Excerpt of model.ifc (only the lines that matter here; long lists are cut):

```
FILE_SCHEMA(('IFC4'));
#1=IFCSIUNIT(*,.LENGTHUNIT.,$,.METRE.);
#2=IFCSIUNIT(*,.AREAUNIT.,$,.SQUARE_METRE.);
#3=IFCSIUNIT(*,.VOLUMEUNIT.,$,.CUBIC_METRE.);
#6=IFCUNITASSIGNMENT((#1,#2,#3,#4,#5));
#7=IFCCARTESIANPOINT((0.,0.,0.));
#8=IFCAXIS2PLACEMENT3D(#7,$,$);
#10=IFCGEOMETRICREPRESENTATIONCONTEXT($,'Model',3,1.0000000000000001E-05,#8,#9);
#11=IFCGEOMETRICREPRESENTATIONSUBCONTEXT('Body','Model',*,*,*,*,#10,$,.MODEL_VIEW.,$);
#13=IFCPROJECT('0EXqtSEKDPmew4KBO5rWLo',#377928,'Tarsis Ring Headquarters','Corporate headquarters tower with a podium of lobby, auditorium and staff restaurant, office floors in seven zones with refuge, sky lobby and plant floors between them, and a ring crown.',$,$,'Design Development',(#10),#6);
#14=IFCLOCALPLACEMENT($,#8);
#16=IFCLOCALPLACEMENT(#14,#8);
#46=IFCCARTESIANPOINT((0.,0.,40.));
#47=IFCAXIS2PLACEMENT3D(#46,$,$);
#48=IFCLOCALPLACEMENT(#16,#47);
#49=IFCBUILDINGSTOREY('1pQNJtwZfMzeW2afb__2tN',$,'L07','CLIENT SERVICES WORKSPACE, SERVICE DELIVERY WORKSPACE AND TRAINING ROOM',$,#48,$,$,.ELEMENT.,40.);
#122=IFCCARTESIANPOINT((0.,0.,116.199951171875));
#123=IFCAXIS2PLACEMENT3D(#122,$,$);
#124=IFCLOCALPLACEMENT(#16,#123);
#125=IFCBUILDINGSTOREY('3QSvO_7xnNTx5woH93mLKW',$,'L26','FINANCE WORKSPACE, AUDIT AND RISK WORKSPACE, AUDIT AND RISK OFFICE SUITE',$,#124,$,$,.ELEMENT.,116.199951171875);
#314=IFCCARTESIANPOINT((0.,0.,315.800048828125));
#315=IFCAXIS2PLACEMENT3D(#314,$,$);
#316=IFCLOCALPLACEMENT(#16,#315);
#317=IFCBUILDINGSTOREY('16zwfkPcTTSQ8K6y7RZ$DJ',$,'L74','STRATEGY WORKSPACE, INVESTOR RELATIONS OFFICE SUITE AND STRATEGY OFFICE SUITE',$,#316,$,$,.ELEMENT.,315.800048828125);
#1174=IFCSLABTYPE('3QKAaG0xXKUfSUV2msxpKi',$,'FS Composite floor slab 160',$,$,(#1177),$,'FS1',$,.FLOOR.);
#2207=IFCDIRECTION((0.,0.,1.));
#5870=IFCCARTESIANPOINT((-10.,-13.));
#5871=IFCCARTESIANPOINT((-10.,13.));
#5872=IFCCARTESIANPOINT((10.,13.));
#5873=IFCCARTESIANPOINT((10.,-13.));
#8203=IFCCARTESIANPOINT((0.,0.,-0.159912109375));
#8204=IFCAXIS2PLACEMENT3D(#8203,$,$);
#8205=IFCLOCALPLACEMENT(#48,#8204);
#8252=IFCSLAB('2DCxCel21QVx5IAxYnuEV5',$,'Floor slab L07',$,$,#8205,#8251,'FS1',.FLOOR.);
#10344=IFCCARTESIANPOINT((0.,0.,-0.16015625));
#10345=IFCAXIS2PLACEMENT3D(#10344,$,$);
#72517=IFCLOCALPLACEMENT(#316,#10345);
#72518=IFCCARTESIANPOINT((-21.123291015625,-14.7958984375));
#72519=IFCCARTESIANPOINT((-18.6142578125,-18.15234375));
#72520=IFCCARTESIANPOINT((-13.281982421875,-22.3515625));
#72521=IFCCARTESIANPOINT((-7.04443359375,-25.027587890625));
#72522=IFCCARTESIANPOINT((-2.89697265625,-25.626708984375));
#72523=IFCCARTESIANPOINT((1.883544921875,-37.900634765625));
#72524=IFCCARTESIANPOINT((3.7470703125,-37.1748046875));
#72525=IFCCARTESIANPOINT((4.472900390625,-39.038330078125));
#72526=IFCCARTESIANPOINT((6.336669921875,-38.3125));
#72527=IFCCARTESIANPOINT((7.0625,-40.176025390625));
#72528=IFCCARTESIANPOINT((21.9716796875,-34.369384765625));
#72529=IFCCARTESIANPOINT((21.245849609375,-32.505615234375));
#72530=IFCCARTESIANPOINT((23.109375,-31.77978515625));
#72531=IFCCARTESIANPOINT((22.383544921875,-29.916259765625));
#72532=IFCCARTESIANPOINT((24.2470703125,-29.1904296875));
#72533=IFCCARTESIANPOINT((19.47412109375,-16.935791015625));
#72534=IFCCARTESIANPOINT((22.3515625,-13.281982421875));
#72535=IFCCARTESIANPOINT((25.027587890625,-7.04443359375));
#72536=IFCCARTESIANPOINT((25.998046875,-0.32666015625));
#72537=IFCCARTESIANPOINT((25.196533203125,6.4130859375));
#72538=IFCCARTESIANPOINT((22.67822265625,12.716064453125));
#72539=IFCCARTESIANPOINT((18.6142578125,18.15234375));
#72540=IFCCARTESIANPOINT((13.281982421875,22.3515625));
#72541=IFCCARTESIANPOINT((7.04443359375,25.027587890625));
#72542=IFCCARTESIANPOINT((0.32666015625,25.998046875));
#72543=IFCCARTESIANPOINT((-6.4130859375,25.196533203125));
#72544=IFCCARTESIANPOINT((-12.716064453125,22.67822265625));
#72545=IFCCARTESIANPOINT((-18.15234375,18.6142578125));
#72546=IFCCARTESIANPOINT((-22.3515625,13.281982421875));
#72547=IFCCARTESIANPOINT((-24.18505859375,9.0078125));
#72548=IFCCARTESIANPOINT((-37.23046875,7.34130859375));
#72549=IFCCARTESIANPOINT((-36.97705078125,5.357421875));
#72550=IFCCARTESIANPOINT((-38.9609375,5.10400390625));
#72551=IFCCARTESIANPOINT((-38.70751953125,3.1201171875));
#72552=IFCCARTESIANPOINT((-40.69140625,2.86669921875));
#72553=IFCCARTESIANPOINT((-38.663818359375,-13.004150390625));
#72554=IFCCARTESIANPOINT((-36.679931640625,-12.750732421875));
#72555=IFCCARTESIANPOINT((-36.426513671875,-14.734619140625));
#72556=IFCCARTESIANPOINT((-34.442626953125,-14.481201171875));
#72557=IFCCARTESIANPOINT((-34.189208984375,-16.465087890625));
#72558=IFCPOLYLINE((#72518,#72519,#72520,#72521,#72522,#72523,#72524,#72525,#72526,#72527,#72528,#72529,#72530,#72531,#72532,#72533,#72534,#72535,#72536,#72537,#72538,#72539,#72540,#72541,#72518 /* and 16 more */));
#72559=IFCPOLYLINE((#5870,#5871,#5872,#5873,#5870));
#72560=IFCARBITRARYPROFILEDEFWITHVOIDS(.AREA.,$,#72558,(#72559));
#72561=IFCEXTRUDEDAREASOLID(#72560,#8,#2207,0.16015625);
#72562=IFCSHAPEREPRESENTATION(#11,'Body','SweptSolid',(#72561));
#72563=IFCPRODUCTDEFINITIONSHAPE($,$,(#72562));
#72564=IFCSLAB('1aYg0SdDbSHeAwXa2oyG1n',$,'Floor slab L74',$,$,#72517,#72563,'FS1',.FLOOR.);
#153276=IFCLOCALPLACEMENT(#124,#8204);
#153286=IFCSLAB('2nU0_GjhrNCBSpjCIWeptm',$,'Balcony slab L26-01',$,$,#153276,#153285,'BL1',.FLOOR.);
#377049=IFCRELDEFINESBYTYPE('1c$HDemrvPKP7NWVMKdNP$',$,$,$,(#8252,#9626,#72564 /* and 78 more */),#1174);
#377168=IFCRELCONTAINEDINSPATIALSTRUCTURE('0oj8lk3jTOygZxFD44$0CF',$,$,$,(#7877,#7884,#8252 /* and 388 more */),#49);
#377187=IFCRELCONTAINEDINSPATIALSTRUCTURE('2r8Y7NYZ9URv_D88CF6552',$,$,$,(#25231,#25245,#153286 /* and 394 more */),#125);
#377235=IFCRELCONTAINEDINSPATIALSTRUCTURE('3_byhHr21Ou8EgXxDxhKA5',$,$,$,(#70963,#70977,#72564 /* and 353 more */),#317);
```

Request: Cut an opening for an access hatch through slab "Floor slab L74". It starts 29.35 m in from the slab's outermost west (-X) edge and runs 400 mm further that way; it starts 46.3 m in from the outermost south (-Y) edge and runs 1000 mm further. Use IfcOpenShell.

```python
import numpy as np
import ifcopenshell
import ifcopenshell.api.feature
import ifcopenshell.api.geometry
import ifcopenshell.api.root
import ifcopenshell.geom
import ifcopenshell.util.placement
import ifcopenshell.util.representation
import ifcopenshell.util.shape
import ifcopenshell.util.unit

model = ifcopenshell.open("model.ifc")
unit_scale = ifcopenshell.util.unit.calculate_unit_scale(model)
settings = ifcopenshell.geom.settings()


def volume(element):
    """Net volume in cubic metres, openings subtracted."""
    shape = ifcopenshell.geom.create_shape(settings, element)
    return ifcopenshell.util.shape.get_volume(shape.geometry)


slab = model.by_guid("1aYg0SdDbSHeAwXa2oyG1n")
before = volume(slab)

# Extent in the slab's own axes, in metres. The edges named are its -X and -Y sides.
slab_shape = ifcopenshell.geom.create_shape(settings, slab)
vertices = ifcopenshell.util.shape.get_vertices(slab_shape.geometry)
x_min, y_min, bottom = vertices.min(axis=0)
top = vertices[:, 2].max()

opening = ifcopenshell.api.root.create_entity(model, ifc_class="IfcOpeningElement", name="Access hatch opening", predefined_type="OPENING")
context = ifcopenshell.util.representation.get_context(model, "Model", "Body", "MODEL_VIEW")
width, depth = 0.4, 1
outline = [(0.0, 0.0), (width, 0.0), (width, depth), (0.0, depth), (0.0, 0.0)]
# Overshoot both faces by 50 mm so the cut is clean.
shape = ifcopenshell.api.geometry.add_slab_representation(
    model, context=context, depth=top - bottom + 0.1, polyline=outline
)
ifcopenshell.api.geometry.assign_representation(model, product=opening, representation=shape)

matrix = ifcopenshell.util.placement.get_local_placement(slab.ObjectPlacement)
matrix[:, 3] = matrix @ np.append(np.array([x_min + 29.35, y_min + 46.3, bottom - 0.05]) / unit_scale, 1.0)
ifcopenshell.api.geometry.edit_object_placement(model, product=opening, matrix=matrix, is_si=False)
ifcopenshell.api.feature.add_feature(model, feature=opening, element=slab)

after = volume(slab)

print(f"slab volume {before:.3f} -> {after:.3f} m3")

model.write("model_v2.ifc")
```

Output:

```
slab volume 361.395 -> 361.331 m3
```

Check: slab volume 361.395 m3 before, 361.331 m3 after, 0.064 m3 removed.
